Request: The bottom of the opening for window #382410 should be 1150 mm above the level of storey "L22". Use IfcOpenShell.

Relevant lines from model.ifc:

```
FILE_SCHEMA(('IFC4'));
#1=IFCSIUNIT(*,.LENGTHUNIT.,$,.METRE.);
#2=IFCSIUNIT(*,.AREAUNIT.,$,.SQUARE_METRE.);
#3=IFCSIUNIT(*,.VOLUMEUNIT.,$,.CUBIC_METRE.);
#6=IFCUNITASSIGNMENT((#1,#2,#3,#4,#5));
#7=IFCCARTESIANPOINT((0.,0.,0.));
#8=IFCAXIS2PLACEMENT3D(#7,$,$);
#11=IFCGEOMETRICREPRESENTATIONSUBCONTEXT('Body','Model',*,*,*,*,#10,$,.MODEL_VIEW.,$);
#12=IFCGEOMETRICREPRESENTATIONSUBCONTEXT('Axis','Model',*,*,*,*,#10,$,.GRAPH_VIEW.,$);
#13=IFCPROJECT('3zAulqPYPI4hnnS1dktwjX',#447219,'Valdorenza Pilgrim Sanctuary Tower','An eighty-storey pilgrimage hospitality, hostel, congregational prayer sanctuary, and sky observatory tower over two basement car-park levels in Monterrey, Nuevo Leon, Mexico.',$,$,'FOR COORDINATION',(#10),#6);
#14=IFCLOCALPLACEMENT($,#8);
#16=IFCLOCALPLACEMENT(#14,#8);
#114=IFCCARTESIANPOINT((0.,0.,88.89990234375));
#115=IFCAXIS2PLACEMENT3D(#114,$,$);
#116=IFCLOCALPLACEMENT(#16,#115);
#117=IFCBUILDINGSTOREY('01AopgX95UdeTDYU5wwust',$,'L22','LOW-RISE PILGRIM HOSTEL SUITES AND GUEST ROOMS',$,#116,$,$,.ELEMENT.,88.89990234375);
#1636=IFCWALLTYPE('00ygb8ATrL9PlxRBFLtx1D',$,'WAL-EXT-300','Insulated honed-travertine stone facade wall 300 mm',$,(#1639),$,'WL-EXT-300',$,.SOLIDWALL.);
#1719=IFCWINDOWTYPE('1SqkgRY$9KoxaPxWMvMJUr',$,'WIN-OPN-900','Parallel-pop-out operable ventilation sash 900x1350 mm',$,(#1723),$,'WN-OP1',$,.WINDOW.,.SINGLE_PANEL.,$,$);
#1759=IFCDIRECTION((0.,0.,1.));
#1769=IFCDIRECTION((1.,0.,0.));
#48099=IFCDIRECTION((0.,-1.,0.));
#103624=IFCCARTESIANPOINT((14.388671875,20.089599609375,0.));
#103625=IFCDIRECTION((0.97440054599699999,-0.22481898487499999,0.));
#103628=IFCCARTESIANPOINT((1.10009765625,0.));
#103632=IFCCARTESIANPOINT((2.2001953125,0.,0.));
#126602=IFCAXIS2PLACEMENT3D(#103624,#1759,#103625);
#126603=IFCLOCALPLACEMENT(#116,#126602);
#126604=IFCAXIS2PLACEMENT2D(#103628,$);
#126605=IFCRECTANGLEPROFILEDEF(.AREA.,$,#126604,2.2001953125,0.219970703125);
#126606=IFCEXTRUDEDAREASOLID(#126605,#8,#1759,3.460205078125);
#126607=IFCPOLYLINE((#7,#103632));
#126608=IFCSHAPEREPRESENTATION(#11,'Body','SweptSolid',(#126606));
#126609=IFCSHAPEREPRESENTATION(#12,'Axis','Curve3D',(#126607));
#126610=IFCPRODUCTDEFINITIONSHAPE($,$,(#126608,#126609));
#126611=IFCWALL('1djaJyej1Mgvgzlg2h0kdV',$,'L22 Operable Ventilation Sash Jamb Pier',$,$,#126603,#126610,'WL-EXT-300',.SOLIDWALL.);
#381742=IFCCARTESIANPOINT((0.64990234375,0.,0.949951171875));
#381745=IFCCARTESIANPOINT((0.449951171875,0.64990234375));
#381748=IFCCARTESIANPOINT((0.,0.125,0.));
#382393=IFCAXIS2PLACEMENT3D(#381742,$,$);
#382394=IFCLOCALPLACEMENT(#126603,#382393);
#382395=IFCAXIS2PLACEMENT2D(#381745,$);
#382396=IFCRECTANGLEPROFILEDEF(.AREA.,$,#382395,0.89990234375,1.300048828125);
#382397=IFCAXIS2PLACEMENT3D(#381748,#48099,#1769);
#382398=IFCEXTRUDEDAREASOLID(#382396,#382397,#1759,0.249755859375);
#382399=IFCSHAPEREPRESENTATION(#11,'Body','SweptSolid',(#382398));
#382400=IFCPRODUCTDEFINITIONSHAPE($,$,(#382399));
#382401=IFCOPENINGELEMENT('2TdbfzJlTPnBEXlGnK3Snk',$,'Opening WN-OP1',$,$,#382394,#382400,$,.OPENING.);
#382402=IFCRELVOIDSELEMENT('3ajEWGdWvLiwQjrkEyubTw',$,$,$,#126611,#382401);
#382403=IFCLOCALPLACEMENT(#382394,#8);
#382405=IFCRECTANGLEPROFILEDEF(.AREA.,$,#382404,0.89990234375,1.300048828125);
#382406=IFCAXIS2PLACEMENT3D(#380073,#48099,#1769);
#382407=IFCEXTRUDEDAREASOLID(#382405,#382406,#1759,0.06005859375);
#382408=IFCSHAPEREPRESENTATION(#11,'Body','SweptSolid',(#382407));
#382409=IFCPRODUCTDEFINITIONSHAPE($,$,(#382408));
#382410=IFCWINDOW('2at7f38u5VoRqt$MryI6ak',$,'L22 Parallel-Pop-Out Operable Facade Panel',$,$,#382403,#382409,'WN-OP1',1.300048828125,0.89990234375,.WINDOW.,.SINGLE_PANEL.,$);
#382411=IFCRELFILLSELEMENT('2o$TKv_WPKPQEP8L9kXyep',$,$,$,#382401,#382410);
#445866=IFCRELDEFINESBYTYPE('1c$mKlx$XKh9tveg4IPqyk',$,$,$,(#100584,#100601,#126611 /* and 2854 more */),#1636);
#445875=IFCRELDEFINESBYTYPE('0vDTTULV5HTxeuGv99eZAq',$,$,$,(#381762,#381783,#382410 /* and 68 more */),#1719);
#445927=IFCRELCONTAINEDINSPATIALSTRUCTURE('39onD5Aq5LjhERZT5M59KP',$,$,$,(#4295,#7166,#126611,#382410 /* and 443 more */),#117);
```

```python
import numpy as np
import ifcopenshell
import ifcopenshell.api.geometry
import ifcopenshell.geom
import ifcopenshell.util.element
import ifcopenshell.util.placement
import ifcopenshell.util.shape
import ifcopenshell.util.unit

model = ifcopenshell.open("model.ifc")
unit_scale = ifcopenshell.util.unit.calculate_unit_scale(model)

window = model.by_guid("2at7f38u5VoRqt$MryI6ak")
opening = window.FillsVoids[0].RelatingOpeningElement
storey = ifcopenshell.util.element.get_container(window, ifc_class="IfcBuildingStorey")
level = ifcopenshell.util.placement.get_local_placement(storey.ObjectPlacement)[2, 3]

# The opening's origin need not be at the sill, so measure its lowest point.
shape = ifcopenshell.geom.create_shape(ifcopenshell.geom.settings(), opening)
bottom = ifcopenshell.util.shape.get_shape_bottom_elevation(shape, shape.geometry) / unit_scale
dz = level + 1.15 / unit_scale - bottom

shift = np.array([0.0, 0.0, dz])
# The window is placed relative to its opening, so it follows when the opening moves.
matrix = ifcopenshell.util.placement.get_local_placement(opening.ObjectPlacement)
matrix[:3, 3] += shift
ifcopenshell.api.geometry.edit_object_placement(
    model, product=opening, matrix=matrix, is_si=False, should_transform_children=True
)

print(f"moved by {dz * unit_scale:+.3f} m")

model.write("model_updated.ifc")
```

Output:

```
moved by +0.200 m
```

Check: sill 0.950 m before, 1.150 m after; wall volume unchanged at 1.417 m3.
